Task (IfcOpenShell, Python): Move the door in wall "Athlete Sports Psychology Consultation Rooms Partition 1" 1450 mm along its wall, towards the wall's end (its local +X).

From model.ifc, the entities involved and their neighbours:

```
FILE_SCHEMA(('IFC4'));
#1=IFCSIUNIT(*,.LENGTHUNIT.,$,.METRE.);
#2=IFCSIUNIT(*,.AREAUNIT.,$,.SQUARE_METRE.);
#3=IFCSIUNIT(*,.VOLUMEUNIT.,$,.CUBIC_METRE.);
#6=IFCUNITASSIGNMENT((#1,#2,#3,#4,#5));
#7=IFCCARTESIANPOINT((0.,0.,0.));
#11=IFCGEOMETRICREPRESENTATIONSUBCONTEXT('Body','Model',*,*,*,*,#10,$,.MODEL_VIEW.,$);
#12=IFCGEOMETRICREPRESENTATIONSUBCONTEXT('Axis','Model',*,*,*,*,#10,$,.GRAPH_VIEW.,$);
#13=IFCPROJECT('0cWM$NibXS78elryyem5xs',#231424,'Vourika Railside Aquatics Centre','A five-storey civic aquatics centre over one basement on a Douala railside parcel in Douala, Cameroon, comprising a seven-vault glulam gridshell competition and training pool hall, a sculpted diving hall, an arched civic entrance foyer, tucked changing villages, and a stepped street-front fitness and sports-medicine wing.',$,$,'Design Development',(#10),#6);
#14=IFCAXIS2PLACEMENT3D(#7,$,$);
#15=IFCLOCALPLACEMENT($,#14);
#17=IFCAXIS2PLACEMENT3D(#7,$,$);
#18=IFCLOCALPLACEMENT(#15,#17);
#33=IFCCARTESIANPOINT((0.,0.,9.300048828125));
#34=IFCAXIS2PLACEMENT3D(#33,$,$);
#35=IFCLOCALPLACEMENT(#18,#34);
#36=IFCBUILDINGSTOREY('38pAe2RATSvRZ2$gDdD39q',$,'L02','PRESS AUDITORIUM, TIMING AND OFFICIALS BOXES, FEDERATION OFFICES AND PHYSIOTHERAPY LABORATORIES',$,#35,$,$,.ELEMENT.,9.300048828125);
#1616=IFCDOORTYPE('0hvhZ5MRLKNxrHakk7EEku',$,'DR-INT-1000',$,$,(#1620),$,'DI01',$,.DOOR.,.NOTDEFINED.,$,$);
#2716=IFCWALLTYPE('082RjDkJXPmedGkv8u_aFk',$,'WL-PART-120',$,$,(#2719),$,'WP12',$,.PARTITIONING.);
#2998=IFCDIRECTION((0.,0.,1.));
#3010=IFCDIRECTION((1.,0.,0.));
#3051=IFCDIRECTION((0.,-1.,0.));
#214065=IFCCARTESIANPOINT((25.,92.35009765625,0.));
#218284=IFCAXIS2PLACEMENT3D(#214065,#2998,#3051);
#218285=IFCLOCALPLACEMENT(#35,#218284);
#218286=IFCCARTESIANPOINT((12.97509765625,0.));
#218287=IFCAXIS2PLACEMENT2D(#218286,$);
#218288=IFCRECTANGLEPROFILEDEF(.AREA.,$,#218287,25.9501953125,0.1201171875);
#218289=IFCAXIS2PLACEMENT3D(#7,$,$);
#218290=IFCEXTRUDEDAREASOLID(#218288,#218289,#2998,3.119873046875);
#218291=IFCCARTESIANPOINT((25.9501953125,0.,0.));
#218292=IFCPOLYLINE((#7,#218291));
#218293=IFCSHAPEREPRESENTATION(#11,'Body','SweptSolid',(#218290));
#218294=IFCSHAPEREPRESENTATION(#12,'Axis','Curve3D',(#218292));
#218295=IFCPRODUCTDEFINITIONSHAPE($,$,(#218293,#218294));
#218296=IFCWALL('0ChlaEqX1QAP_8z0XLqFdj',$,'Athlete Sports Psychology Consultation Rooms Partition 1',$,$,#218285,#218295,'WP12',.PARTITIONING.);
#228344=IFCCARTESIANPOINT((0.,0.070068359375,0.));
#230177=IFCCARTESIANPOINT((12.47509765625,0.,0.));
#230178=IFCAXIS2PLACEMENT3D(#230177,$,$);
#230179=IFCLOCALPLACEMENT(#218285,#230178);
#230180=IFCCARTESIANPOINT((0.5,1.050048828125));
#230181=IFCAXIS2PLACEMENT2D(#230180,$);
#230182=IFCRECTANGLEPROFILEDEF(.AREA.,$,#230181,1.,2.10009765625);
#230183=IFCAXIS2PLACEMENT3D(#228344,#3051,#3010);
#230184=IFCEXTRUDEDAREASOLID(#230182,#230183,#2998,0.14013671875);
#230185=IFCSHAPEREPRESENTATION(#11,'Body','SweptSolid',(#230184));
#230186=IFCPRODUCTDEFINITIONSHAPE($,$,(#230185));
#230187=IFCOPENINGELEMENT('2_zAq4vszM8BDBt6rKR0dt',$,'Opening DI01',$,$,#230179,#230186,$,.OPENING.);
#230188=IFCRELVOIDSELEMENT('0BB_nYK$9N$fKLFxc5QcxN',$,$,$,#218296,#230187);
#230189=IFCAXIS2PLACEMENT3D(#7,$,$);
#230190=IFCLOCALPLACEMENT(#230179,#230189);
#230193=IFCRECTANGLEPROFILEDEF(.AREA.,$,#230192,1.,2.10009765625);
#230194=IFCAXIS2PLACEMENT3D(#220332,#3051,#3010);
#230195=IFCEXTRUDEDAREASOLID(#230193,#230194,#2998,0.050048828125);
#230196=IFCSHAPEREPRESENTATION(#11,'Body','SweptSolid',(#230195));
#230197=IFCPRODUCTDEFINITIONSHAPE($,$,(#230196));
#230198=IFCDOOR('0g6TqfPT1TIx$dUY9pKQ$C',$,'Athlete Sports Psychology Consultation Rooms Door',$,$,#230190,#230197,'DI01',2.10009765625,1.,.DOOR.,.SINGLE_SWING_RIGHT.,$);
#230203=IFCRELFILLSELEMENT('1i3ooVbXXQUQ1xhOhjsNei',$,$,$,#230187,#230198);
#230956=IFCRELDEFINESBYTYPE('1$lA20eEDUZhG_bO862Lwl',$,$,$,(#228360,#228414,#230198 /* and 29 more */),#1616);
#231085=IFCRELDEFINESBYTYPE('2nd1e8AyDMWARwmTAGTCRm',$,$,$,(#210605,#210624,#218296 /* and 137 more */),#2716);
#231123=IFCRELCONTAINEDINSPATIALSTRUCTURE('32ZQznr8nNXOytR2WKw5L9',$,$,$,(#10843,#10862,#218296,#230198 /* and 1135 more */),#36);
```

```python
import ifcopenshell
import ifcopenshell.api.geometry
import ifcopenshell.util.placement
import ifcopenshell.util.unit

model = ifcopenshell.open("model.ifc")
unit_scale = ifcopenshell.util.unit.calculate_unit_scale(model)

door = model.by_id(230198)
opening = door.FillsVoids[0].RelatingOpeningElement
wall = opening.VoidsElements[0].RelatingBuildingElement

wall_matrix = ifcopenshell.util.placement.get_local_placement(wall.ObjectPlacement)
shift = wall_matrix[:3, 0] * 1.45 / unit_scale
before = ifcopenshell.util.placement.get_local_placement(door.ObjectPlacement)[:3, 3].copy()

# The door is placed relative to its opening, so it follows when the opening moves.
matrix = ifcopenshell.util.placement.get_local_placement(opening.ObjectPlacement)
matrix[:3, 3] += shift
ifcopenshell.api.geometry.edit_object_placement(
    model, product=opening, matrix=matrix, is_si=False, should_transform_children=True
)

after = ifcopenshell.util.placement.get_local_placement(door.ObjectPlacement)[:3, 3]
print("door moved by", (after - before).round(3) + 0.0)

model.write("model_rev.ifc")
```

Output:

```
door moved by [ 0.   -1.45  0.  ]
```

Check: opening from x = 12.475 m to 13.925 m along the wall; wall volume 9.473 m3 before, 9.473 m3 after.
